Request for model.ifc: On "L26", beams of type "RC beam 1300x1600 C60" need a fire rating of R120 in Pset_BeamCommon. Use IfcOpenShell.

First a look at what the model holds.

```python
import ifcopenshell
import ifcopenshell.util.element

model = ifcopenshell.open("model.ifc")
print(model.schema)
storey = next(s for s in model.by_type("IfcBuildingStorey") if s.Name == "L26")
beams = [e for e in ifcopenshell.util.element.get_decomposition(storey) if e.is_a("IfcBeam")]
seen = {}
for e in beams:
    element_type = ifcopenshell.util.element.get_type(e)
    key = (element_type.Name if element_type != e and element_type else None, ifcopenshell.util.element.get_pset(e, "Pset_BeamCommon", "FireRating"))
    seen[key] = seen.get(key, 0) + 1
for (name, value), count in sorted(seen.items(), key=str):
    print(count, "x", name, "|", value)
```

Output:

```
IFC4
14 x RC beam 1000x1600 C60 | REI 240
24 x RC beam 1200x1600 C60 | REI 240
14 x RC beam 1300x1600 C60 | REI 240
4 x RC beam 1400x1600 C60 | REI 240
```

```python
import ifcopenshell
import ifcopenshell.api.pset
import ifcopenshell.util.element

model = ifcopenshell.open("model.ifc")

storey = next(s for s in model.by_type("IfcBuildingStorey") if s.Name == "L26")
beams = [e for e in ifcopenshell.util.element.get_decomposition(storey) if e.is_a("IfcBeam")]

count = 0
for e in beams:
    element_type = ifcopenshell.util.element.get_type(e)
    if element_type in (None, e) or element_type.Name != "RC beam 1300x1600 C60":
        continue
    found = ifcopenshell.util.element.get_pset(e, "Pset_BeamCommon", should_inherit=False)
    if found:
        pset = model.by_id(found["id"])
        if len(ifcopenshell.util.element.get_elements_by_pset(pset)) > 1:
            pset = ifcopenshell.api.pset.unshare_pset(model, products=[e], pset=pset)[0]
    else:
        pset = ifcopenshell.api.pset.add_pset(model, product=e, name="Pset_BeamCommon")
    ifcopenshell.api.pset.edit_pset(model, pset=pset, properties={"FireRating": "R120"})
    count += 1

print(count, "beams updated")

model.write("model_edited.ifc")
```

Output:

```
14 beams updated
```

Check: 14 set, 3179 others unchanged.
